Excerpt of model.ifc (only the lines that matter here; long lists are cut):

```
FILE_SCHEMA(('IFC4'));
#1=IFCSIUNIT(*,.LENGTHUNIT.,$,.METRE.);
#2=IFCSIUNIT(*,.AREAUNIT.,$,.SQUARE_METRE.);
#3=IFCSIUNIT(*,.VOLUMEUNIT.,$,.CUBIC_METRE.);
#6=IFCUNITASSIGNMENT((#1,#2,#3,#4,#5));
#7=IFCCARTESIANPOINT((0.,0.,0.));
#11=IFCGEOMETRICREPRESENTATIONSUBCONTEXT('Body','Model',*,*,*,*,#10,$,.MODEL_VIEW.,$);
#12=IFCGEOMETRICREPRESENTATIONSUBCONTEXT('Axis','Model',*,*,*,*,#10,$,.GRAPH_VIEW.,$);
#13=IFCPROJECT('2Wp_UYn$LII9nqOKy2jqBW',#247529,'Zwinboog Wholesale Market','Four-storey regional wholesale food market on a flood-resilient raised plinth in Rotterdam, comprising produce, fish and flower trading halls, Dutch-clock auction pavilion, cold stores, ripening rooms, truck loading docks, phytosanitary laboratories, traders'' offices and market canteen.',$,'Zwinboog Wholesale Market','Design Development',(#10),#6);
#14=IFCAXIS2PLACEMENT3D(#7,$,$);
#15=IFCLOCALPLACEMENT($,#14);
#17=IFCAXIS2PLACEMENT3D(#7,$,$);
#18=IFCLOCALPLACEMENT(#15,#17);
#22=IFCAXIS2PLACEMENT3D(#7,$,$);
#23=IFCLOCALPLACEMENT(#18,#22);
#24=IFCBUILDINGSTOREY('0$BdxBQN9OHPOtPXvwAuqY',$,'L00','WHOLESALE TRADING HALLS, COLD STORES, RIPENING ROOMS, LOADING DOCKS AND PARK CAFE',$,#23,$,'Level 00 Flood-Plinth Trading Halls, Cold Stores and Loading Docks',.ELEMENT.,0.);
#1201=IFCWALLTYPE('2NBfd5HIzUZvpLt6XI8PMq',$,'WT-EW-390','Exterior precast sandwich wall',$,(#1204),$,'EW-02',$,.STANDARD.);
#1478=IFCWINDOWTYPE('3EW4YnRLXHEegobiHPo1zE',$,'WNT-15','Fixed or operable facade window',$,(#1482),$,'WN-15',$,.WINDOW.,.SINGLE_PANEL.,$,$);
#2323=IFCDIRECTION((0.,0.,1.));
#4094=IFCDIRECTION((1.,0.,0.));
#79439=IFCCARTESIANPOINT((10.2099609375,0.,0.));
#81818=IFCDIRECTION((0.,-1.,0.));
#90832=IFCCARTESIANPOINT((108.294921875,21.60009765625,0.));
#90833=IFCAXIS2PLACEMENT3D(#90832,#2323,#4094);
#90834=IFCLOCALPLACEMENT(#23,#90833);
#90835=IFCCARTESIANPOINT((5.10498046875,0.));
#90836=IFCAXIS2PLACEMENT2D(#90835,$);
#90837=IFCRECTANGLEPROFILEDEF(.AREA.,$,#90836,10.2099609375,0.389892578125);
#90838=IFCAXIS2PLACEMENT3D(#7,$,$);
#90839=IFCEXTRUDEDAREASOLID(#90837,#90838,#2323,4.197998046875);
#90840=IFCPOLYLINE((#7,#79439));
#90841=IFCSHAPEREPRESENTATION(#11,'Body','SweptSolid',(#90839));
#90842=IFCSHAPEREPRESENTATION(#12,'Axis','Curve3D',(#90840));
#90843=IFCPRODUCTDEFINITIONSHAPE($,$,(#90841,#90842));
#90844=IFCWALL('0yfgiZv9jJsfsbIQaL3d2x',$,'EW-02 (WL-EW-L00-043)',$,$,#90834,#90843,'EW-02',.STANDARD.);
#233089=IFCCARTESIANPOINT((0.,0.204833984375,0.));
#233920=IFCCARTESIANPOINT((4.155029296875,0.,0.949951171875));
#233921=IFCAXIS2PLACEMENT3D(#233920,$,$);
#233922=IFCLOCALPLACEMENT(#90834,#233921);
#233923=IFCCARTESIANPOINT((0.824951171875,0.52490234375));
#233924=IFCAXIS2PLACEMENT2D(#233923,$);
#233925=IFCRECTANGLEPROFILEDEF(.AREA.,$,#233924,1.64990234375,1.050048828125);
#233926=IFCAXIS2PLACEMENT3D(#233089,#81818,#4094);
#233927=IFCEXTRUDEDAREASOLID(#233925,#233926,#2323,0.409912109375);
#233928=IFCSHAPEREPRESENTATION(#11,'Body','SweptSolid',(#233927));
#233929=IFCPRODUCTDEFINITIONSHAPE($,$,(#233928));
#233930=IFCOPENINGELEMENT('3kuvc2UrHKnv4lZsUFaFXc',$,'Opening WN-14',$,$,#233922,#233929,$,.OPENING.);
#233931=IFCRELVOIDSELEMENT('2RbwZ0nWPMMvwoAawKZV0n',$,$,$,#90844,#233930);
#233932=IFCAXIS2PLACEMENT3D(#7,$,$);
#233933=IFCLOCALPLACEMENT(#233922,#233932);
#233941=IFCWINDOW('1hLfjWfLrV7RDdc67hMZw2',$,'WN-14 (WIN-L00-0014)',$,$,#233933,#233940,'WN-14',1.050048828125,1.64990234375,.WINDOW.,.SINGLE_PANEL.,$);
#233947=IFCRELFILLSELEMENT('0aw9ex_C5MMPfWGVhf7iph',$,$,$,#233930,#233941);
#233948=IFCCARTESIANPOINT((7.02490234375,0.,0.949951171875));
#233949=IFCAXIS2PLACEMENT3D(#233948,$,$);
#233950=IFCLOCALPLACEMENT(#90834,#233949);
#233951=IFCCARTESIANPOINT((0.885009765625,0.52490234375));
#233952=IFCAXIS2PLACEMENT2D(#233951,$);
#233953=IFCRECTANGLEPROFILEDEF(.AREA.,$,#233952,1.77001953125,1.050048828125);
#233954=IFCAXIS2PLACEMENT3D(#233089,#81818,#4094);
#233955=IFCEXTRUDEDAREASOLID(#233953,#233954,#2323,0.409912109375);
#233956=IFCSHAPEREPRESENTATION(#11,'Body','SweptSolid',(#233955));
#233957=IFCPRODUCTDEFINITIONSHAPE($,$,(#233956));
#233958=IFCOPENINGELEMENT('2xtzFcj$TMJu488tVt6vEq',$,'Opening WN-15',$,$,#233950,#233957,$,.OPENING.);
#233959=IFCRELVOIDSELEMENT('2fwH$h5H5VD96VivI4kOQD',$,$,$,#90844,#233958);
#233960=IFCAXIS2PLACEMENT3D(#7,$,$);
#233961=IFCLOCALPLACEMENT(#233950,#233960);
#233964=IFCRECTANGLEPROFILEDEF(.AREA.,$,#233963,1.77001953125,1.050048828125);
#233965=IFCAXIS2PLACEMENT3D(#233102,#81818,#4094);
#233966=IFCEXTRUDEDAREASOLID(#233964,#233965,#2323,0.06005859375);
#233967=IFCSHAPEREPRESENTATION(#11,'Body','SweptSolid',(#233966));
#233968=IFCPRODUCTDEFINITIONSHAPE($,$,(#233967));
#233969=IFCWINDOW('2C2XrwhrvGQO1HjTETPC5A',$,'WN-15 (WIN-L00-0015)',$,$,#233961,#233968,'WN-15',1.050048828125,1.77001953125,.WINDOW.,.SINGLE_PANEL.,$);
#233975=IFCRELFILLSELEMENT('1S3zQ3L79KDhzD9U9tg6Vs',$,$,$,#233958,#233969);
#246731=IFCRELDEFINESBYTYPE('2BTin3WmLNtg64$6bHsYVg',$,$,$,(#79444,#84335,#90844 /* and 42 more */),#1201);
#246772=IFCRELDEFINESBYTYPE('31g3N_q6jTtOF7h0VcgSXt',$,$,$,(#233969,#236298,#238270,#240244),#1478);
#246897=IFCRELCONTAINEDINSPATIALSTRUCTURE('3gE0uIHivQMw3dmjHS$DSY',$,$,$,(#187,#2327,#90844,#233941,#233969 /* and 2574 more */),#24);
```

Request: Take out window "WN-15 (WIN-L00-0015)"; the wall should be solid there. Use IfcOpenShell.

```python
import ifcopenshell
import ifcopenshell.api.feature
import ifcopenshell.api.root
import ifcopenshell.geom
import ifcopenshell.util.shape

model = ifcopenshell.open("model.ifc")
settings = ifcopenshell.geom.settings()


def volume(element):
    """Net volume in cubic metres, openings subtracted."""
    shape = ifcopenshell.geom.create_shape(settings, element)
    return ifcopenshell.util.shape.get_volume(shape.geometry)


window = model.by_id(233969)
opening = window.FillsVoids[0].RelatingOpeningElement
wall = opening.VoidsElements[0].RelatingBuildingElement
before = volume(wall)

ifcopenshell.api.root.remove_product(model, product=window)
ifcopenshell.api.feature.remove_feature(model, feature=opening)

after = volume(wall)

print(f"wall volume {before:.3f} -> {after:.3f} m3")

model.write("model_v2.ifc")
```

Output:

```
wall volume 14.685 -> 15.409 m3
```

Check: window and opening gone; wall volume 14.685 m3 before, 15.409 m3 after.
